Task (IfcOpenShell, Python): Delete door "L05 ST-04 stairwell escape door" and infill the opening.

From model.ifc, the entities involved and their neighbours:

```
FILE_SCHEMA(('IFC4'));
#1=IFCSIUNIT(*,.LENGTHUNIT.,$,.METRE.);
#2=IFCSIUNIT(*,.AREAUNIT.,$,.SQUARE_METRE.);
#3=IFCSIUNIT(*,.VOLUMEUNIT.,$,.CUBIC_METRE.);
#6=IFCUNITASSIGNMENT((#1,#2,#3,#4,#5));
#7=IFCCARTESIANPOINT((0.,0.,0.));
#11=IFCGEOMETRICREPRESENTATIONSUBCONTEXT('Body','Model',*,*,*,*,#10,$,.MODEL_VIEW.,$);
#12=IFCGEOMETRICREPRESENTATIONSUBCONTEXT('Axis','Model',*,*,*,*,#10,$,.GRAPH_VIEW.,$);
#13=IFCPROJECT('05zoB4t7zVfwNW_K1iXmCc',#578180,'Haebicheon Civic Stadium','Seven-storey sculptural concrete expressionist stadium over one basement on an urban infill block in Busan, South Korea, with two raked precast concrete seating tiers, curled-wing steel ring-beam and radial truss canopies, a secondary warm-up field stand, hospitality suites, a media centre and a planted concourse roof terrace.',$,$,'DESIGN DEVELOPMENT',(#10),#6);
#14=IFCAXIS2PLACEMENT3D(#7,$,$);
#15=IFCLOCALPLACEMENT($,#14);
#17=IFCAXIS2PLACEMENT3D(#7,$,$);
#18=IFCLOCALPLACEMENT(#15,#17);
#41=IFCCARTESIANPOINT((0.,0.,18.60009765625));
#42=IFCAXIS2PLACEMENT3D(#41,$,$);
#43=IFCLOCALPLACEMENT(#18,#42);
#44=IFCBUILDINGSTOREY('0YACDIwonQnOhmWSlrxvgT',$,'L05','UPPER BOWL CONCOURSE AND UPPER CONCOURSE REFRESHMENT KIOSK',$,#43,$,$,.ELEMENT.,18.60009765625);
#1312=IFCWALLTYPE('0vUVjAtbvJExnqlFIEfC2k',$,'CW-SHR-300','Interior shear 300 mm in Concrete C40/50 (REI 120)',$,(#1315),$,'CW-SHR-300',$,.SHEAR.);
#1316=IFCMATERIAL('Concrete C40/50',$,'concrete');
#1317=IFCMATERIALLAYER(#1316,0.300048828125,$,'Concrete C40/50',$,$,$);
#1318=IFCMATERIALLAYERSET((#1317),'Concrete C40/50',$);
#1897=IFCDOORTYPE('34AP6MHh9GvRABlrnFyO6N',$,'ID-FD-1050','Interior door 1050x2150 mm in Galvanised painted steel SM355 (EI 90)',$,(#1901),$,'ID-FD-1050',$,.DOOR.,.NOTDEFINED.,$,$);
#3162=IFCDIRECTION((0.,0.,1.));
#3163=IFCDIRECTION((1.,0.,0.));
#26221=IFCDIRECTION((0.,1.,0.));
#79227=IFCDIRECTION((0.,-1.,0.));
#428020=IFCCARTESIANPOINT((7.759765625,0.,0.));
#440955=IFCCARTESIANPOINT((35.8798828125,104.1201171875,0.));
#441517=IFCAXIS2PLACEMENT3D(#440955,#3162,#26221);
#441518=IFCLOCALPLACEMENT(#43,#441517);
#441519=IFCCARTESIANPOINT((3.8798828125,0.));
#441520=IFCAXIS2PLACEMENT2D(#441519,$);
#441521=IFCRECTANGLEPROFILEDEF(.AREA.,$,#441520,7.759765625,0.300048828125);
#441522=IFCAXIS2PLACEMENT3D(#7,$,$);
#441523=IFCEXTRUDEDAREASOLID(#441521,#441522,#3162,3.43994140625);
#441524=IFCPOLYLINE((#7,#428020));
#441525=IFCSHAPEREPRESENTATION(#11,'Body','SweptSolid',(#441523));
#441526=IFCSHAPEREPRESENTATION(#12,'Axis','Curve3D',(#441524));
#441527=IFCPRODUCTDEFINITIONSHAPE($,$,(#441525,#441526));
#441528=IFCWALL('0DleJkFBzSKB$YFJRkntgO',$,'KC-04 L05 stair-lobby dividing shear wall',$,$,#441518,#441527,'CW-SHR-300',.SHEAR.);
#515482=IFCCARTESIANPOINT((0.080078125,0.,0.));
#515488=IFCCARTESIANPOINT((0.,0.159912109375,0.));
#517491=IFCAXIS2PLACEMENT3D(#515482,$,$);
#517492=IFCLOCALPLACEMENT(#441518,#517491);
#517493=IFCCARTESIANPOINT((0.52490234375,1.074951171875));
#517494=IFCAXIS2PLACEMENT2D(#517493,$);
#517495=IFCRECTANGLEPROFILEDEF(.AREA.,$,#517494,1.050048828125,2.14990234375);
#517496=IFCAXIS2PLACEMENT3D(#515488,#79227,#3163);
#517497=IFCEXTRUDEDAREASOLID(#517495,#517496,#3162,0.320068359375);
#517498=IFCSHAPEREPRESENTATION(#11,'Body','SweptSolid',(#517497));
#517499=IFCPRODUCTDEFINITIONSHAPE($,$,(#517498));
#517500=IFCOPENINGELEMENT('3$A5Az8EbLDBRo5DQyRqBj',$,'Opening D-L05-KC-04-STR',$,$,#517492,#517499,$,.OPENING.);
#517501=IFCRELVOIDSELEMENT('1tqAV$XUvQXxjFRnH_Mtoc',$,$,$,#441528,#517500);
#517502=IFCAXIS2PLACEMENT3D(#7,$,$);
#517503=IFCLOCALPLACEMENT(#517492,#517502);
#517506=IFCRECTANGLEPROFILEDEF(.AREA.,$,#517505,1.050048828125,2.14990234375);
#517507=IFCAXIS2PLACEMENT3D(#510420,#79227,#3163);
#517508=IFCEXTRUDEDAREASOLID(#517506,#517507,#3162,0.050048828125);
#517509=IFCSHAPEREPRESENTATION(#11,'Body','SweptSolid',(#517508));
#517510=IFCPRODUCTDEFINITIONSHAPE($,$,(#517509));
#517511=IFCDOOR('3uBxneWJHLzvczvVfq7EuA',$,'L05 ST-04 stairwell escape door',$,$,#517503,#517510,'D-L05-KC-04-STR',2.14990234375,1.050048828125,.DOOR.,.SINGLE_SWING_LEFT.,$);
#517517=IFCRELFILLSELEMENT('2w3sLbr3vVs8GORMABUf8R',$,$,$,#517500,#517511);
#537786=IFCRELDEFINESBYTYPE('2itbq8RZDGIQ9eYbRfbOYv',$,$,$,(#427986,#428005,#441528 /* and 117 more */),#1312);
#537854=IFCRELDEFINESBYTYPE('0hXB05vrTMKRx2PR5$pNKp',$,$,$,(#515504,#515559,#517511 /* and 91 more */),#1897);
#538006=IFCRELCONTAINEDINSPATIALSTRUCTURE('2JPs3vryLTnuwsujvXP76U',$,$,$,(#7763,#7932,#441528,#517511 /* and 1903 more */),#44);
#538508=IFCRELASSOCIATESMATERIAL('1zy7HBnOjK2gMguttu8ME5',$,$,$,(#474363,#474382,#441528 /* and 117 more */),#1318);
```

```python
import ifcopenshell
import ifcopenshell.api.feature
import ifcopenshell.api.root
import ifcopenshell.geom
import ifcopenshell.util.shape

model = ifcopenshell.open("model.ifc")
settings = ifcopenshell.geom.settings()


def volume(element):
    """Net volume in cubic metres, openings subtracted."""
    shape = ifcopenshell.geom.create_shape(settings, element)
    return ifcopenshell.util.shape.get_volume(shape.geometry)


door = model.by_id(517511)
opening = door.FillsVoids[0].RelatingOpeningElement
wall = opening.VoidsElements[0].RelatingBuildingElement
before = volume(wall)

ifcopenshell.api.root.remove_product(model, product=door)
ifcopenshell.api.feature.remove_feature(model, feature=opening)

after = volume(wall)

print(f"wall volume {before:.3f} -> {after:.3f} m3")

model.write("model_edited.ifc")
```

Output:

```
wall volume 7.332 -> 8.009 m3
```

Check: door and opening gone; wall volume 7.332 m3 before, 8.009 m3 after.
